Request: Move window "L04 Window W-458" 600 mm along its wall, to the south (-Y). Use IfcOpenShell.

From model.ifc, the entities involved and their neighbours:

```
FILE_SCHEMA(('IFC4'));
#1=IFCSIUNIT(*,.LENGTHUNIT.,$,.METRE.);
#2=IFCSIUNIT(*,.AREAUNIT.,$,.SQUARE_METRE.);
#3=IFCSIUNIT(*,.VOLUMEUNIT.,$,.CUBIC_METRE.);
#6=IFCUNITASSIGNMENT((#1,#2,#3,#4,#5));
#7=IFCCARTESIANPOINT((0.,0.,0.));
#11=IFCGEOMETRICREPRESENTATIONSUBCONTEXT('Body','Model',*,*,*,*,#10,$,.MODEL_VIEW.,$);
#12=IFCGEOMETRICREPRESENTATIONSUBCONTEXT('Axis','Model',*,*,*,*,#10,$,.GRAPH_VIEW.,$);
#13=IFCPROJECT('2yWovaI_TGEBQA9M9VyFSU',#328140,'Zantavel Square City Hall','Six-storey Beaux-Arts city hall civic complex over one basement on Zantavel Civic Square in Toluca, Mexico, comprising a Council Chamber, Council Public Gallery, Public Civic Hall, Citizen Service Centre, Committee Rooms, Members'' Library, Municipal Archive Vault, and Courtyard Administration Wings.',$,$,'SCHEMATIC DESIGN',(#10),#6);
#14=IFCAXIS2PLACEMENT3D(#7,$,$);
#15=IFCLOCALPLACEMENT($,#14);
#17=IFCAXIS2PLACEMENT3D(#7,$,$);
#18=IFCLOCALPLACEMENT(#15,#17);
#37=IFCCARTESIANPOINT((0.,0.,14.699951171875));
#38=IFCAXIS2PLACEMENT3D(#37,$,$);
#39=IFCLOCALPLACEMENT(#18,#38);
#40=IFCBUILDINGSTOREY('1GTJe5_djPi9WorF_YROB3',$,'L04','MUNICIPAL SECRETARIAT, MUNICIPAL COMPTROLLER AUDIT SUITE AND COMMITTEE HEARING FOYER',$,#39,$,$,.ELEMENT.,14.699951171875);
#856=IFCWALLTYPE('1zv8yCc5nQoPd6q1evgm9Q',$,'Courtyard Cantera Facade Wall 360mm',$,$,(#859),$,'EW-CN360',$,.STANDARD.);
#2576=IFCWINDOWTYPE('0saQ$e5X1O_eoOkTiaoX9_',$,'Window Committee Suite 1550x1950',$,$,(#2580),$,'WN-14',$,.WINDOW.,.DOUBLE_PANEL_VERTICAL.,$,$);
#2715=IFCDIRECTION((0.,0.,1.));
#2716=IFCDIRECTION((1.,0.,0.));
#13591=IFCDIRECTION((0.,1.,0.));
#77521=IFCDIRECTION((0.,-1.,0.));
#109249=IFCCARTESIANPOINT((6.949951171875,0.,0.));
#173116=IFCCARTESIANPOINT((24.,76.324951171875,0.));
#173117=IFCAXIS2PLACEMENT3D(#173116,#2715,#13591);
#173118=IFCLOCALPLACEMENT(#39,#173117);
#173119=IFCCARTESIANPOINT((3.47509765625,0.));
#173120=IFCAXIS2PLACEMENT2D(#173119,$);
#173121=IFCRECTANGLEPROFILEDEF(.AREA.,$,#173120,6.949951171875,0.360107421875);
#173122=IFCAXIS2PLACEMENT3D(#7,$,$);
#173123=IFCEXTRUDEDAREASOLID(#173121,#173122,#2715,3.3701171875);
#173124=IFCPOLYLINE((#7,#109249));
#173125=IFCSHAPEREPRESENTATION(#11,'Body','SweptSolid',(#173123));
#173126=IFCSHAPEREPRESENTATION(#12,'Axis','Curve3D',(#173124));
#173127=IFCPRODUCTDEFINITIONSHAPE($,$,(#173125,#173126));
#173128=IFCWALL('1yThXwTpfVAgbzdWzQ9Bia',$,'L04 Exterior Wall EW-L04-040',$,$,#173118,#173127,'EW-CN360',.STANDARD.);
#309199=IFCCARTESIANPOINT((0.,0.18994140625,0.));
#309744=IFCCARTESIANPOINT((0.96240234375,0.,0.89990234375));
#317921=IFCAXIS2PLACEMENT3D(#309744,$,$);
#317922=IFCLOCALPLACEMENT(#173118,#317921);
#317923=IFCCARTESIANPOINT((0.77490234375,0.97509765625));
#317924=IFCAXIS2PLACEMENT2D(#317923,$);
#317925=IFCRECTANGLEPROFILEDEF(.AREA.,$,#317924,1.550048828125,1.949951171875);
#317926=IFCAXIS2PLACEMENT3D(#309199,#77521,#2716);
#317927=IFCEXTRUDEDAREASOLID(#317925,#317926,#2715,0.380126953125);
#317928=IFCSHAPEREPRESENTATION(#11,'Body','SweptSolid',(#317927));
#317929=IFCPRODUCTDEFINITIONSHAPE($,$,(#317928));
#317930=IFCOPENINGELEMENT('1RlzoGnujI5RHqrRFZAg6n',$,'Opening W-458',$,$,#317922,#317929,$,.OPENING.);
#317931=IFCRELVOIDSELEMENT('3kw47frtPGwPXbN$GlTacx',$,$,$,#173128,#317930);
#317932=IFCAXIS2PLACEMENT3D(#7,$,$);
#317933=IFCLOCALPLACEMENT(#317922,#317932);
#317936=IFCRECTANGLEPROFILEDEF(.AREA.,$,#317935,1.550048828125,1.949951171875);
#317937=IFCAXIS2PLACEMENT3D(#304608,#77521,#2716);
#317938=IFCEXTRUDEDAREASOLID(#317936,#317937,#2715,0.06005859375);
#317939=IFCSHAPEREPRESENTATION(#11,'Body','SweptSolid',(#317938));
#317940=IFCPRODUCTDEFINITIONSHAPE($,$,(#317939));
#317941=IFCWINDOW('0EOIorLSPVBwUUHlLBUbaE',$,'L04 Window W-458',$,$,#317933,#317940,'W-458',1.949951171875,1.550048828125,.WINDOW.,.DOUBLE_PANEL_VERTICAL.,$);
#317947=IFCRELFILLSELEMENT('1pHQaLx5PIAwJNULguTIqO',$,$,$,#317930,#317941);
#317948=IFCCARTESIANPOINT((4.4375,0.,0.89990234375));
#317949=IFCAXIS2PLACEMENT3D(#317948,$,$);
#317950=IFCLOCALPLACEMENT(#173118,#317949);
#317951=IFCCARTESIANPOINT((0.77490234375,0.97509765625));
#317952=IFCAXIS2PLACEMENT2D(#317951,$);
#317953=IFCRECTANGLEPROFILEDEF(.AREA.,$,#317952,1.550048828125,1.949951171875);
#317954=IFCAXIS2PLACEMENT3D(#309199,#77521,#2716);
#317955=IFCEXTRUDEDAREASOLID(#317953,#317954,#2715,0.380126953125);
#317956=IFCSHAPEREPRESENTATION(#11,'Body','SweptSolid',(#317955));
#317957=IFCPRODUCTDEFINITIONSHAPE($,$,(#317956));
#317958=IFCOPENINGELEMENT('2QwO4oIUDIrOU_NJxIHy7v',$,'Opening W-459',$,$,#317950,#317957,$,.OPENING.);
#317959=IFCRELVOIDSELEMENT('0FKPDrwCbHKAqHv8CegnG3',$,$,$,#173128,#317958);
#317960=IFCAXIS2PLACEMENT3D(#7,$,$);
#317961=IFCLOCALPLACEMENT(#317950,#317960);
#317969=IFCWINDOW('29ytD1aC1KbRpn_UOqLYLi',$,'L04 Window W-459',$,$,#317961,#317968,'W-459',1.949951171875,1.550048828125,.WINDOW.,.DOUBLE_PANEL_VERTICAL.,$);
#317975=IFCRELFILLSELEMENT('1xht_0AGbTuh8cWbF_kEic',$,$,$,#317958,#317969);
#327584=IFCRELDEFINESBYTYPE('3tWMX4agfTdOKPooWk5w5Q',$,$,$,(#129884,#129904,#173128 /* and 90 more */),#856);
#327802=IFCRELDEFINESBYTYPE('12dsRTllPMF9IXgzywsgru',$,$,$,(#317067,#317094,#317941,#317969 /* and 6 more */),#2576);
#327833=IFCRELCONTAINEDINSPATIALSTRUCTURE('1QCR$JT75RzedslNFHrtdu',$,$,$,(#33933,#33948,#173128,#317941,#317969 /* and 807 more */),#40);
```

```python
import ifcopenshell
import ifcopenshell.api.geometry
import ifcopenshell.util.placement

model = ifcopenshell.open("model.ifc")

window = model.by_guid("0EOIorLSPVBwUUHlLBUbaE")
opening = window.FillsVoids[0].RelatingOpeningElement
wall = opening.VoidsElements[0].RelatingBuildingElement

wall_matrix = ifcopenshell.util.placement.get_local_placement(wall.ObjectPlacement)
shift = wall_matrix[:3, 0] * -0.6
before = ifcopenshell.util.placement.get_local_placement(window.ObjectPlacement)[:3, 3].copy()

# The window is placed relative to its opening, so it follows when the opening moves.
matrix = ifcopenshell.util.placement.get_local_placement(opening.ObjectPlacement)
matrix[:3, 3] += shift
ifcopenshell.api.geometry.edit_object_placement(
    model, product=opening, matrix=matrix, is_si=False, should_transform_children=True
)

after = ifcopenshell.util.placement.get_local_placement(window.ObjectPlacement)[:3, 3]
print("window moved by", (after - before).round(3) + 0.0)

model.write("model_updated.ifc")
```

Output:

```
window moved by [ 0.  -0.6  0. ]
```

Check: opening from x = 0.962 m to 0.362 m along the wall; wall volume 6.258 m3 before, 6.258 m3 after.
